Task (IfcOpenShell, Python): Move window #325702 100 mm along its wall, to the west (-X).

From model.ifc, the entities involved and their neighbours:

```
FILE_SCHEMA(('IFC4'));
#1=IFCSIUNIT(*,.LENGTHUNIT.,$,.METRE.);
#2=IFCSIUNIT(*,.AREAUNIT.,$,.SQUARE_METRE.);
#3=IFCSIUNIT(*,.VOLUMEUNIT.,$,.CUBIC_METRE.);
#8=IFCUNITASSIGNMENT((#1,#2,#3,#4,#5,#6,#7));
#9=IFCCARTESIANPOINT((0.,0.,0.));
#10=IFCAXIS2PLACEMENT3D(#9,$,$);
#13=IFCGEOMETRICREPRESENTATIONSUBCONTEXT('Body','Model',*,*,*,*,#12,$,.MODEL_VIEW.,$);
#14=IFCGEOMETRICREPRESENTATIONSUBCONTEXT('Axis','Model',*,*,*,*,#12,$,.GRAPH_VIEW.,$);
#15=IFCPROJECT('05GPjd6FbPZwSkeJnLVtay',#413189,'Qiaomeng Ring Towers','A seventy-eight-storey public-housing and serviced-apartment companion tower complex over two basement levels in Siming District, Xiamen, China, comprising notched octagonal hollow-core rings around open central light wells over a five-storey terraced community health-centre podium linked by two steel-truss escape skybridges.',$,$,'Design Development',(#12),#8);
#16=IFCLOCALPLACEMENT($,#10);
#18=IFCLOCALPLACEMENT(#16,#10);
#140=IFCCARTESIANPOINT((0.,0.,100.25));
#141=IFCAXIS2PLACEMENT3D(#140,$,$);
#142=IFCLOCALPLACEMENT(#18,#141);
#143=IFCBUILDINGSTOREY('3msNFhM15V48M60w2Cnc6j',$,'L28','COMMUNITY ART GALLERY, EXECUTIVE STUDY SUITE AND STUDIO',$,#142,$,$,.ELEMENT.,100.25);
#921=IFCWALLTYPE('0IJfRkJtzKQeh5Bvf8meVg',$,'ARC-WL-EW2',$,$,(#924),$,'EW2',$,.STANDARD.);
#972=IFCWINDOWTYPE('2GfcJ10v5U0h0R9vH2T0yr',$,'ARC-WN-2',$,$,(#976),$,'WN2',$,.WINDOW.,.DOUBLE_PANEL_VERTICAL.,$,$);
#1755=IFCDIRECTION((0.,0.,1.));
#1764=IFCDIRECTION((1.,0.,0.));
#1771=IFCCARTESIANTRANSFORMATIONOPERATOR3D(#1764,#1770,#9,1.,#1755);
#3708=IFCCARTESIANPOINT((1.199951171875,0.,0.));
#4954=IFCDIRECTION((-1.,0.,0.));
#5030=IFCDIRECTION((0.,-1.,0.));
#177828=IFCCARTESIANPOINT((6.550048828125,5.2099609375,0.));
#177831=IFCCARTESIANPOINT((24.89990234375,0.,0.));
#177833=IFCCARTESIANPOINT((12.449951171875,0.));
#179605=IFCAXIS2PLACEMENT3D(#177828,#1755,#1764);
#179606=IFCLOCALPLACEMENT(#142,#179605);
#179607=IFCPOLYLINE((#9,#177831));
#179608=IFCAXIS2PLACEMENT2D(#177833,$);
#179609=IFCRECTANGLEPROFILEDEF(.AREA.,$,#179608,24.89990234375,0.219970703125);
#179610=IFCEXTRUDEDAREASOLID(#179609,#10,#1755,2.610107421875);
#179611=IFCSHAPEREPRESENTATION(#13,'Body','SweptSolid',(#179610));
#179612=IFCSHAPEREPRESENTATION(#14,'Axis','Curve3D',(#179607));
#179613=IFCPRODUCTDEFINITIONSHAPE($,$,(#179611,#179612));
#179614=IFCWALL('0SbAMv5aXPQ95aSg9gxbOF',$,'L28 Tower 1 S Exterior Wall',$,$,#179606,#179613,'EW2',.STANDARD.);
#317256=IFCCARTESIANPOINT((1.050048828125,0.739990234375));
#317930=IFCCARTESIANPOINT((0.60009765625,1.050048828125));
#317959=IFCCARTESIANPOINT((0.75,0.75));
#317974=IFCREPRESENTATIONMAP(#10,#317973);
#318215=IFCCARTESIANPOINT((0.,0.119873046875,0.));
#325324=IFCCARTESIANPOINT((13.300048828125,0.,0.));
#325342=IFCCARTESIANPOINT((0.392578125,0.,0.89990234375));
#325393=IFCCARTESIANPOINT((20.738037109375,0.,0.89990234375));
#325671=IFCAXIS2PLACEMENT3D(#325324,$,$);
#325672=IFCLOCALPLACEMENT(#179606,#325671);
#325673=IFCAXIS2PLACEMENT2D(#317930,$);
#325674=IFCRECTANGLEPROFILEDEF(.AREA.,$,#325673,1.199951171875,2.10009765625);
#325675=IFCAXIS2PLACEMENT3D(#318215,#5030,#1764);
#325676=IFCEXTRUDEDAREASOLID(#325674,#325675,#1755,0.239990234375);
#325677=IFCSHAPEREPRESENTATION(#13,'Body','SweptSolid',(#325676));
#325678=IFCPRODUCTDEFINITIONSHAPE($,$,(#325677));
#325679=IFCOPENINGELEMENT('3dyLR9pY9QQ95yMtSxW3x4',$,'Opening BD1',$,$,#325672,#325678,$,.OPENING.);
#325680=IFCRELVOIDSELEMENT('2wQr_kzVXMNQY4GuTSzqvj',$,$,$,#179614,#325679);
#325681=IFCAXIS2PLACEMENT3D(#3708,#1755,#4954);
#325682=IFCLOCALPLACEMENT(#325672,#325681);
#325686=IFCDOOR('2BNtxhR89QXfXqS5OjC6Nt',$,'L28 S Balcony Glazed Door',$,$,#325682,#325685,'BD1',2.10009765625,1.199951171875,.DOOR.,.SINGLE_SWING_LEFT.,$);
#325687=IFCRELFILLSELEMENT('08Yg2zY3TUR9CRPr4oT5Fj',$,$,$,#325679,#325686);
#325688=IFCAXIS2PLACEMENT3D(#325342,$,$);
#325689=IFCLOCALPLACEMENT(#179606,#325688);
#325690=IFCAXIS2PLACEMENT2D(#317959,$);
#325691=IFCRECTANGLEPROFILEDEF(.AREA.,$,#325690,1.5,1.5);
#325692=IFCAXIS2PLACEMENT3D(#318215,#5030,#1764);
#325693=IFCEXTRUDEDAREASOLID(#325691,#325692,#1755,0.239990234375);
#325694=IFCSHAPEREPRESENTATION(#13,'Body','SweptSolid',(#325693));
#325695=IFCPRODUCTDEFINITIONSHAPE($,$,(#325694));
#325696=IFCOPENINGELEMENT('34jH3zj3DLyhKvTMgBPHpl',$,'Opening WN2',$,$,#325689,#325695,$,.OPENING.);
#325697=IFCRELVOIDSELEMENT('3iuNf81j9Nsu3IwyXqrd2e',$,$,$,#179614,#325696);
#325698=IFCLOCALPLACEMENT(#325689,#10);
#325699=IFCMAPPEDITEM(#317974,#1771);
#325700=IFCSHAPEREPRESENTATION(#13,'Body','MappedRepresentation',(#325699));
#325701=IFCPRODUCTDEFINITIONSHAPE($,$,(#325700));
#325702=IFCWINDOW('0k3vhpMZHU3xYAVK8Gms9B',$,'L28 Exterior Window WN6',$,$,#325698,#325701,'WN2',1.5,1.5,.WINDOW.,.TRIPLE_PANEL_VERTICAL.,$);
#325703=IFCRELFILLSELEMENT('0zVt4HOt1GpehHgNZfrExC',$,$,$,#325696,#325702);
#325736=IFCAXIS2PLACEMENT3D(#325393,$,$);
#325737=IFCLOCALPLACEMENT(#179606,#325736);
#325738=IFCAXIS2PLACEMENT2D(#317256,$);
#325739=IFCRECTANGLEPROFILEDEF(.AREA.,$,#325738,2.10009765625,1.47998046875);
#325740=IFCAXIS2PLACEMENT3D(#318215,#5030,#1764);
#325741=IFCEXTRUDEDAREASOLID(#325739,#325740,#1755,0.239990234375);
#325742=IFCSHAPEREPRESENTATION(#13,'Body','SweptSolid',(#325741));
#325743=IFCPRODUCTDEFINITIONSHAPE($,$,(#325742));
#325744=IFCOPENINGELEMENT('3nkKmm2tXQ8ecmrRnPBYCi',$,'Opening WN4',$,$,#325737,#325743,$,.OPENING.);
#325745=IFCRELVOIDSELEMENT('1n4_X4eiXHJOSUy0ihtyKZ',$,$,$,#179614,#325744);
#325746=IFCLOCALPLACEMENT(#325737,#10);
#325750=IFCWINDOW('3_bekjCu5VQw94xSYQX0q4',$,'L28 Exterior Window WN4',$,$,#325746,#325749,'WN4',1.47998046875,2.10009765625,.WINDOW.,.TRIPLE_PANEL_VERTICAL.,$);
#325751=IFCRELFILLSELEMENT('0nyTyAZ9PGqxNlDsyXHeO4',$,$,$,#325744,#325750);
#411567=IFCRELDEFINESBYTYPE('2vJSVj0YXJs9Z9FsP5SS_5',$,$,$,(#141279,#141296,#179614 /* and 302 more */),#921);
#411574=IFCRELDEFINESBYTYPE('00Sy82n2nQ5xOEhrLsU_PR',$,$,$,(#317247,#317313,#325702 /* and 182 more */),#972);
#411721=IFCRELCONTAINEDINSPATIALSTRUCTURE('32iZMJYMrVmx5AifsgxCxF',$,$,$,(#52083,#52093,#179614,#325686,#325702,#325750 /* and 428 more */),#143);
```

```python
import ifcopenshell
import ifcopenshell.api.geometry
import ifcopenshell.util.placement
import ifcopenshell.util.unit

model = ifcopenshell.open("model.ifc")
unit_scale = ifcopenshell.util.unit.calculate_unit_scale(model)

window = model.by_guid("0k3vhpMZHU3xYAVK8Gms9B")
opening = window.FillsVoids[0].RelatingOpeningElement
wall = opening.VoidsElements[0].RelatingBuildingElement

wall_matrix = ifcopenshell.util.placement.get_local_placement(wall.ObjectPlacement)
shift = wall_matrix[:3, 0] * -0.1 / unit_scale
before = ifcopenshell.util.placement.get_local_placement(window.ObjectPlacement)[:3, 3].copy()

# The window is placed relative to its opening, so it follows when the opening moves.
matrix = ifcopenshell.util.placement.get_local_placement(opening.ObjectPlacement)
matrix[:3, 3] += shift
ifcopenshell.api.geometry.edit_object_placement(
    model, product=opening, matrix=matrix, is_si=False, should_transform_children=True
)

after = ifcopenshell.util.placement.get_local_placement(window.ObjectPlacement)[:3, 3]
print("window moved by", (after - before).round(3) + 0.0)

model.write("model-out.ifc")
```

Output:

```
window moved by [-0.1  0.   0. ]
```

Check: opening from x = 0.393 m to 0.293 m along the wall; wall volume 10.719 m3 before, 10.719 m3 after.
